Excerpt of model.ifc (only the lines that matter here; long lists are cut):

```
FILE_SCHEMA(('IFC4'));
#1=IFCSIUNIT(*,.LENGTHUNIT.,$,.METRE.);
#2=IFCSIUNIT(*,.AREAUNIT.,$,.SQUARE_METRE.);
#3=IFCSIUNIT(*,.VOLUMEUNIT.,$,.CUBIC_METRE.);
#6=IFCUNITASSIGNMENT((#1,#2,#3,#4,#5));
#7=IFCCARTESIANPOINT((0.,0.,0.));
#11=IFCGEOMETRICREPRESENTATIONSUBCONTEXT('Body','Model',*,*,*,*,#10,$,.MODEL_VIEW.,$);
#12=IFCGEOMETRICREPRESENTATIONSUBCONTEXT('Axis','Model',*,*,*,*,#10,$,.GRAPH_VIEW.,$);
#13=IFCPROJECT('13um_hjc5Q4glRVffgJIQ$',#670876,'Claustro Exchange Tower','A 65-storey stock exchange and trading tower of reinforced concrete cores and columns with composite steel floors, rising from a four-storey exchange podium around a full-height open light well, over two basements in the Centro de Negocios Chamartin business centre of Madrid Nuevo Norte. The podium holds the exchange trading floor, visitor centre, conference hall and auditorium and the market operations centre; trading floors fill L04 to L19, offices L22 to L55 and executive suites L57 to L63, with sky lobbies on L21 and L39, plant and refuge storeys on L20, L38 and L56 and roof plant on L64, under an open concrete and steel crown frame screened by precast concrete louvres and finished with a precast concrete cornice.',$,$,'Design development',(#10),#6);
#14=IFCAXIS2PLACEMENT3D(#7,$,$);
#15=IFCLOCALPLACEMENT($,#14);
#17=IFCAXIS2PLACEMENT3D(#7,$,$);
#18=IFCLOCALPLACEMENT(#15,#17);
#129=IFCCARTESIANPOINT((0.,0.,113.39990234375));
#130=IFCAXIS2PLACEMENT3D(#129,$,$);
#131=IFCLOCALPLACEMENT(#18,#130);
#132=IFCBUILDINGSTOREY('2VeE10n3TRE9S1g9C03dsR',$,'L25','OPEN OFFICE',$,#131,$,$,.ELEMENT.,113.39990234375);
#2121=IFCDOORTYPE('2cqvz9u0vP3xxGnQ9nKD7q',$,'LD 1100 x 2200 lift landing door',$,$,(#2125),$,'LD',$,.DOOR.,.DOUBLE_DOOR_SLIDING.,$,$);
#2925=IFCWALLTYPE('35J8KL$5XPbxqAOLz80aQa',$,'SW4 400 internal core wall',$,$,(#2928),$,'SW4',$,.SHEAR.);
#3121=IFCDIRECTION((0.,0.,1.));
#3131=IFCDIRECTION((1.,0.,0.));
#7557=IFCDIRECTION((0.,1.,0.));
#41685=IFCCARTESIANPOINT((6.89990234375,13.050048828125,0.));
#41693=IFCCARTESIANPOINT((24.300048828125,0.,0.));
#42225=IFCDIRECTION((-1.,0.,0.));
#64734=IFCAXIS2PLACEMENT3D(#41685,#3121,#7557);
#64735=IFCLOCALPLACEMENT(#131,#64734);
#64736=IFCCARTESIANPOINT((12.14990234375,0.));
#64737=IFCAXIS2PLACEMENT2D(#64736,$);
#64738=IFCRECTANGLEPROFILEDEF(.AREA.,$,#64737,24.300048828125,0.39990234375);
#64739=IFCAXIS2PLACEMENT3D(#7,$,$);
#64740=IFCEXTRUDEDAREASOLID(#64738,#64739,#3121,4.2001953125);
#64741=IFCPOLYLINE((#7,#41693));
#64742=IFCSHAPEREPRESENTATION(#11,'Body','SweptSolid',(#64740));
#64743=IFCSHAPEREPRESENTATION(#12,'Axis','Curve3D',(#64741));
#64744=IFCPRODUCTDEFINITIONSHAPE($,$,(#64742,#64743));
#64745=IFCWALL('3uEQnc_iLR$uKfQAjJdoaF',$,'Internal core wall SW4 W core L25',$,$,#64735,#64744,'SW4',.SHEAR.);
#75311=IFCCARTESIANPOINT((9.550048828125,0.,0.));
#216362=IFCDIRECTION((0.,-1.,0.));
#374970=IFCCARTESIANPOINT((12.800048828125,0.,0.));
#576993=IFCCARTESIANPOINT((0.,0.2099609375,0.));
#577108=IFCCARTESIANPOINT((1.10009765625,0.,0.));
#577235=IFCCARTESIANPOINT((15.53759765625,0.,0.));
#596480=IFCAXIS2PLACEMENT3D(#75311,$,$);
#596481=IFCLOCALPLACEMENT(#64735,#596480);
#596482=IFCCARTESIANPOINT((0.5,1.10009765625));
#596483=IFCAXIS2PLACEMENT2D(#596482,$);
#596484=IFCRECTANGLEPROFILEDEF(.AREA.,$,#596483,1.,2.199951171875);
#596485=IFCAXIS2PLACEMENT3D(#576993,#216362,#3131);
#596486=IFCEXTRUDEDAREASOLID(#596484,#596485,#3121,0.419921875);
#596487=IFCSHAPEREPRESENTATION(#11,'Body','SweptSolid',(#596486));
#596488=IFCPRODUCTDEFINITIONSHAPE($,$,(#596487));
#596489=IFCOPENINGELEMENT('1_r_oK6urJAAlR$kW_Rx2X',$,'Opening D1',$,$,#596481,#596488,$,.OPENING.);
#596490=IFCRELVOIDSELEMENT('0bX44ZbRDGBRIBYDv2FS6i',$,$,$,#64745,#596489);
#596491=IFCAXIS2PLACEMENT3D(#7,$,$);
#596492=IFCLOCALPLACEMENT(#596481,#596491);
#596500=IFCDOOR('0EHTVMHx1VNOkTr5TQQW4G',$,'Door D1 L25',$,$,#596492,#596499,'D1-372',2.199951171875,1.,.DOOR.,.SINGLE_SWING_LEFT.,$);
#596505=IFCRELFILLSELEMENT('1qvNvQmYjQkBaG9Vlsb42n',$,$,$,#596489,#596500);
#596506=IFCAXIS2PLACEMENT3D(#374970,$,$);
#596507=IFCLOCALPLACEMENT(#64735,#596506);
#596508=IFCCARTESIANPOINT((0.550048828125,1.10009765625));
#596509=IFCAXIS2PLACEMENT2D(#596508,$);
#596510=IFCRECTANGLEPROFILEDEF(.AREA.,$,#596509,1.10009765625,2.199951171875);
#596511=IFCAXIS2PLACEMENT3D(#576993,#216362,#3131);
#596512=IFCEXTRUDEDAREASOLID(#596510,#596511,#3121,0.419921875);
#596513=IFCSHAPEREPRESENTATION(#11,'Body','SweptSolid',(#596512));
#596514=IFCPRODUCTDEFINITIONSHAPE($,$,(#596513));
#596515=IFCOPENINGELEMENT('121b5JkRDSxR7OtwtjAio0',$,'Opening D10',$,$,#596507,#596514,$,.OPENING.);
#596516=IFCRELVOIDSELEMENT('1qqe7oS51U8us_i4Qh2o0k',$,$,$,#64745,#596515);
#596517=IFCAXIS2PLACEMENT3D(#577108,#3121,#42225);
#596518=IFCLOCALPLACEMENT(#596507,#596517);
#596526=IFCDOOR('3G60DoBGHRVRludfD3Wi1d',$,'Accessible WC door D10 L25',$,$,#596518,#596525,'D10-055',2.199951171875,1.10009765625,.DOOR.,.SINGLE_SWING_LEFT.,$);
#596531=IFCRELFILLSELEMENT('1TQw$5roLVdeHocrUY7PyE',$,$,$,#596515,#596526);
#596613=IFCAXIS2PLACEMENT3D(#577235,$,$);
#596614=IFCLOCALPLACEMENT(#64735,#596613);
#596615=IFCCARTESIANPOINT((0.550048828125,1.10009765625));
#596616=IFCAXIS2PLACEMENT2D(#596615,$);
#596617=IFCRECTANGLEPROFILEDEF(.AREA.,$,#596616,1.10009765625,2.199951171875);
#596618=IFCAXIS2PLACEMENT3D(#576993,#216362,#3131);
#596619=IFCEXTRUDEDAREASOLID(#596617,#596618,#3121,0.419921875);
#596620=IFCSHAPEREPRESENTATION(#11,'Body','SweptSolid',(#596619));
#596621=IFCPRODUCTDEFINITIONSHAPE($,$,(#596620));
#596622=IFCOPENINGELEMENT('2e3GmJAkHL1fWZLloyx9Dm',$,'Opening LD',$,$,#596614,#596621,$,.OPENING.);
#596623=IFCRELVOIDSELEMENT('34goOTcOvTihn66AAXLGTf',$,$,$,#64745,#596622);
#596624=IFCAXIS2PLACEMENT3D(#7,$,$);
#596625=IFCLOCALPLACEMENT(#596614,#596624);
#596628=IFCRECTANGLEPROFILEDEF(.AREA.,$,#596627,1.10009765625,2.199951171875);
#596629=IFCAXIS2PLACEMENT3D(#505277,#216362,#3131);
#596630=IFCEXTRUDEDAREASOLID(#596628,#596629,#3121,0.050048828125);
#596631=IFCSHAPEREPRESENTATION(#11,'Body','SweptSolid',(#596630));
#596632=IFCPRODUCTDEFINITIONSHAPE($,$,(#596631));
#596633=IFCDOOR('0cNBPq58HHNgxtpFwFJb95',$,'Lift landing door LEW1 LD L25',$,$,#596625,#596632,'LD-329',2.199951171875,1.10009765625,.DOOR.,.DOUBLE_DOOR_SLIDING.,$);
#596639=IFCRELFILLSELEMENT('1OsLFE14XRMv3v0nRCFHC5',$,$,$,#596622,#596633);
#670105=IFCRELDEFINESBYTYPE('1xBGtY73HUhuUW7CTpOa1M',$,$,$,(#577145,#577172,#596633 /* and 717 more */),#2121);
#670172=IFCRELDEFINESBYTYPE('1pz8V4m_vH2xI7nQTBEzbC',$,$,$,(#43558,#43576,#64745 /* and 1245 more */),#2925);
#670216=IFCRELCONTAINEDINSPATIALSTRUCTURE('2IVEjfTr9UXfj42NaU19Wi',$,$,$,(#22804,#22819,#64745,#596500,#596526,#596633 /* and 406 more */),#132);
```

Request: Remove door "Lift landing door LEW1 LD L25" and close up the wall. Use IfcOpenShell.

```python
import ifcopenshell
import ifcopenshell.api.feature
import ifcopenshell.api.root
import ifcopenshell.geom
import ifcopenshell.util.shape

model = ifcopenshell.open("model.ifc")
settings = ifcopenshell.geom.settings()


def volume(element):
    """Net volume in cubic metres, openings subtracted."""
    shape = ifcopenshell.geom.create_shape(settings, element)
    return ifcopenshell.util.shape.get_volume(shape.geometry)


door = model.by_guid("0cNBPq58HHNgxtpFwFJb95")
opening = door.FillsVoids[0].RelatingOpeningElement
wall = opening.VoidsElements[0].RelatingBuildingElement
before = volume(wall)

ifcopenshell.api.root.remove_product(model, product=door)
ifcopenshell.api.feature.remove_feature(model, feature=opening)

after = volume(wall)

print(f"wall volume {before:.3f} -> {after:.3f} m3")

model.write("model_rev.ifc")
```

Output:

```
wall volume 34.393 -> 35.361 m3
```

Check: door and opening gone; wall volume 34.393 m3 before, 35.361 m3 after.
